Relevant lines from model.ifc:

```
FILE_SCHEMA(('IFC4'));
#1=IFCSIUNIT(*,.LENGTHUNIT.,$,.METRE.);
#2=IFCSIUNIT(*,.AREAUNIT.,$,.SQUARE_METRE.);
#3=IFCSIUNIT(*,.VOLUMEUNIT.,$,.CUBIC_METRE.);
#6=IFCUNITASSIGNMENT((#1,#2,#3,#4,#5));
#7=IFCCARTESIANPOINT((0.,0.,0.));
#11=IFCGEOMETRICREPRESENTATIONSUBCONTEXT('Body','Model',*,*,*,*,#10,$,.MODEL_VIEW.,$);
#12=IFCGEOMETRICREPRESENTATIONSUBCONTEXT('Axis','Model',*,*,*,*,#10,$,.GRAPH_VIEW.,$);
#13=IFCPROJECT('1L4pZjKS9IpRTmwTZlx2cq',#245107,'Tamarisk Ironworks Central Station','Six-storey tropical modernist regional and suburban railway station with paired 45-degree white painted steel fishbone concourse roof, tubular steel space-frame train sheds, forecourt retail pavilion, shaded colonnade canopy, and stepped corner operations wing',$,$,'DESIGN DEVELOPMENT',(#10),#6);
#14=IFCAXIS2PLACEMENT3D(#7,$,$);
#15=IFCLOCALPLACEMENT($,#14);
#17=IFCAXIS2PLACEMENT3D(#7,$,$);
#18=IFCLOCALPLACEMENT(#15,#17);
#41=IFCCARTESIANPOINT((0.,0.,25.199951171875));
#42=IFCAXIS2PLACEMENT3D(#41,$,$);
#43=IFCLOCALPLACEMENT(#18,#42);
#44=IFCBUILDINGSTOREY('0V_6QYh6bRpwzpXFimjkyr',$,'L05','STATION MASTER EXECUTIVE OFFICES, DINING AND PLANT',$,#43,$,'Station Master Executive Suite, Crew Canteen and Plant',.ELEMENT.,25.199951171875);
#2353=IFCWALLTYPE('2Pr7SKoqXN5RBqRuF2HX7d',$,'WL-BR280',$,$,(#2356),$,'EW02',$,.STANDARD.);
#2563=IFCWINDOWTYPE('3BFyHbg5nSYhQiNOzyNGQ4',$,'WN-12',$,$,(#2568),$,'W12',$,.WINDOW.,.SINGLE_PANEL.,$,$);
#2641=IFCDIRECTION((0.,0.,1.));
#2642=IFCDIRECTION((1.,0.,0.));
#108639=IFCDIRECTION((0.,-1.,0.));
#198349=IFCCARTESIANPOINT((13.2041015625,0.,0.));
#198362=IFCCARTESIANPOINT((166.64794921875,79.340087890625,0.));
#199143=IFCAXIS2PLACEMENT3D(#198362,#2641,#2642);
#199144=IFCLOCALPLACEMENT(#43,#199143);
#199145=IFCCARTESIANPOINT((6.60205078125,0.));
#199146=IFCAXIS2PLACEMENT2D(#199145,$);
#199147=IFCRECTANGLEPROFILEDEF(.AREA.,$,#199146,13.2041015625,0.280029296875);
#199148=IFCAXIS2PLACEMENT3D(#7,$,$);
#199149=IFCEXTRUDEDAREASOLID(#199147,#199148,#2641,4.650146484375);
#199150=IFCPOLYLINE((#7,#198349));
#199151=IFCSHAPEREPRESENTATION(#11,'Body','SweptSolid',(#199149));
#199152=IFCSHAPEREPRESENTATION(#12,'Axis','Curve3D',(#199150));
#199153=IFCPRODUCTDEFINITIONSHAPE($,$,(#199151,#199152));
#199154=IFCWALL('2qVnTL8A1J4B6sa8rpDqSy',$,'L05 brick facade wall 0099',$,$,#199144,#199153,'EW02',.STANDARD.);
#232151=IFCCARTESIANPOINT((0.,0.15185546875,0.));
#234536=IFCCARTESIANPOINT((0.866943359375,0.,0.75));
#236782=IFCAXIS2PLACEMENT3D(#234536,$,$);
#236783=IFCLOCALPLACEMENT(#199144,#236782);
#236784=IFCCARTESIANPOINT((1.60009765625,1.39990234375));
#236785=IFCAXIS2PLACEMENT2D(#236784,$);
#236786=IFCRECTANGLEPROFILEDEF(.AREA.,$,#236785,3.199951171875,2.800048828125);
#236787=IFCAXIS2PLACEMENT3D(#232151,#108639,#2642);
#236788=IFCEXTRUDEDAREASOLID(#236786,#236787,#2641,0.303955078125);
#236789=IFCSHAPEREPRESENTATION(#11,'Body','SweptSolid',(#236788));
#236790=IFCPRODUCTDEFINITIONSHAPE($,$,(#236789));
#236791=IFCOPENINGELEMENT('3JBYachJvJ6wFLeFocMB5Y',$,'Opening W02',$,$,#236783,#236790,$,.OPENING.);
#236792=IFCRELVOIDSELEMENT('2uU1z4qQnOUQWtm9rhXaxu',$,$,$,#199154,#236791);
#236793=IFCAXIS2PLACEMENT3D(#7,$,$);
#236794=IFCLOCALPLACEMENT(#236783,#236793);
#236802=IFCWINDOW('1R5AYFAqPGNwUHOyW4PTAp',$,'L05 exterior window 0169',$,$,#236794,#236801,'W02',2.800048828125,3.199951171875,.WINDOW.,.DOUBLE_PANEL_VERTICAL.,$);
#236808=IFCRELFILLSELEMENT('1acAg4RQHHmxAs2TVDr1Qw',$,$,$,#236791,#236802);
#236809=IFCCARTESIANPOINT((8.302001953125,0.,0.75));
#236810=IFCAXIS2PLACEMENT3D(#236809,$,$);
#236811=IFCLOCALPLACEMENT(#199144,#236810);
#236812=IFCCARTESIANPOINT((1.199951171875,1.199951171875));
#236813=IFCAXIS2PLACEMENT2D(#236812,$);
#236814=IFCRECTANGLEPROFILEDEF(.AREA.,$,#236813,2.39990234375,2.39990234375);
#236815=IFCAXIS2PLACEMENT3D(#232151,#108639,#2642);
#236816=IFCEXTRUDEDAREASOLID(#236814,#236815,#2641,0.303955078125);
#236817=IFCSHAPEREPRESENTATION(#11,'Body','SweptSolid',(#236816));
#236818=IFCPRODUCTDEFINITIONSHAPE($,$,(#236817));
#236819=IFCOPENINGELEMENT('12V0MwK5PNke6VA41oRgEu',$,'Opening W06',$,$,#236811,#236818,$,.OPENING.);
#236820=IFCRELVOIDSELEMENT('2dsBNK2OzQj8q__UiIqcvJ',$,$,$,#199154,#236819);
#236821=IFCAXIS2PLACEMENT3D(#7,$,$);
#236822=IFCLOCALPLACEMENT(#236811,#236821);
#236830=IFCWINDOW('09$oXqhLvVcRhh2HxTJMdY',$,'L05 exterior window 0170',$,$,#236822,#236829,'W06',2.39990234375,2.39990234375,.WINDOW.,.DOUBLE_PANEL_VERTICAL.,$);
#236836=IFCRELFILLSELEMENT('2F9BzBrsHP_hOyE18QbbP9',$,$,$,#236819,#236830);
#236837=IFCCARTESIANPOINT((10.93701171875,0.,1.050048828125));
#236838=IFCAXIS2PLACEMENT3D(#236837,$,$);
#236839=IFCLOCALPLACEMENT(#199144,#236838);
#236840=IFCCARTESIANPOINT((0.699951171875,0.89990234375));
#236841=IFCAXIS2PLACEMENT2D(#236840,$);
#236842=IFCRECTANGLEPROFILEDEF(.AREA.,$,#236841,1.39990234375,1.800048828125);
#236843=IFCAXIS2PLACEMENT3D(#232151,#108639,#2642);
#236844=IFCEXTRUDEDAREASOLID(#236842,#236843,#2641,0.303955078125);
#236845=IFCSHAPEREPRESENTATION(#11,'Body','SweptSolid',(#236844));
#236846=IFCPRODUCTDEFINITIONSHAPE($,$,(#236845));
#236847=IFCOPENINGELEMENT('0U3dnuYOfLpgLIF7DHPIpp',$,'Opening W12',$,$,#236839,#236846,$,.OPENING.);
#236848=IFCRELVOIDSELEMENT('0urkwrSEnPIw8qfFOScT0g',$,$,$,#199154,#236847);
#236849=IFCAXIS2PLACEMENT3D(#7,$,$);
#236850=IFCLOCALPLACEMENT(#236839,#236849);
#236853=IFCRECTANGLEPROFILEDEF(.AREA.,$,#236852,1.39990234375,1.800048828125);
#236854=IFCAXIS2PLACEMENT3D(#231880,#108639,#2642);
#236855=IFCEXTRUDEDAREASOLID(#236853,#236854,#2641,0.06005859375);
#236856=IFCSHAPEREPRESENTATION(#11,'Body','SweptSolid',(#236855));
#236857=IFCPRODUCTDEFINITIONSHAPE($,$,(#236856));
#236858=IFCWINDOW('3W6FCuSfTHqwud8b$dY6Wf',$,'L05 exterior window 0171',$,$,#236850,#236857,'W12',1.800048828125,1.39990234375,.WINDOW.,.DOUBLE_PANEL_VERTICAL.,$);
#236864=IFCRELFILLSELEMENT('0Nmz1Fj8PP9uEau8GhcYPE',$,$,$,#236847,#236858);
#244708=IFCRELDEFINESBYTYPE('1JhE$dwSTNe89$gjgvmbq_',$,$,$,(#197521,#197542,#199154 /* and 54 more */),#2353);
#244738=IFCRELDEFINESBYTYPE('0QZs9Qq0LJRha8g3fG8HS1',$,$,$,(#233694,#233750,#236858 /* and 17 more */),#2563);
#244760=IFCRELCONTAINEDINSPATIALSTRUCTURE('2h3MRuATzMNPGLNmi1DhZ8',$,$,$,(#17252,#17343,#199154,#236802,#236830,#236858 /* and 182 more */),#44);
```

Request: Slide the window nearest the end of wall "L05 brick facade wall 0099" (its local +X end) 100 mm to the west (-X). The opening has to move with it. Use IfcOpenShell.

```python
import ifcopenshell
import ifcopenshell.api.geometry
import ifcopenshell.util.placement

model = ifcopenshell.open("model.ifc")

window = model.by_guid("3W6FCuSfTHqwud8b$dY6Wf")
opening = window.FillsVoids[0].RelatingOpeningElement
wall = opening.VoidsElements[0].RelatingBuildingElement

wall_matrix = ifcopenshell.util.placement.get_local_placement(wall.ObjectPlacement)
shift = wall_matrix[:3, 0] * -0.1
before = ifcopenshell.util.placement.get_local_placement(window.ObjectPlacement)[:3, 3].copy()

# The window is placed relative to its opening, so it follows when the opening moves.
matrix = ifcopenshell.util.placement.get_local_placement(opening.ObjectPlacement)
matrix[:3, 3] += shift
ifcopenshell.api.geometry.edit_object_placement(
    model, product=opening, matrix=matrix, is_si=False, should_transform_children=True
)

after = ifcopenshell.util.placement.get_local_placement(window.ObjectPlacement)[:3, 3]
print("window moved by", (after - before).round(3) + 0.0)

model.write("model_edited.ifc")
```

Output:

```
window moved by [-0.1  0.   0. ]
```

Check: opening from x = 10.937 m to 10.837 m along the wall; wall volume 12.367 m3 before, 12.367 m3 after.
